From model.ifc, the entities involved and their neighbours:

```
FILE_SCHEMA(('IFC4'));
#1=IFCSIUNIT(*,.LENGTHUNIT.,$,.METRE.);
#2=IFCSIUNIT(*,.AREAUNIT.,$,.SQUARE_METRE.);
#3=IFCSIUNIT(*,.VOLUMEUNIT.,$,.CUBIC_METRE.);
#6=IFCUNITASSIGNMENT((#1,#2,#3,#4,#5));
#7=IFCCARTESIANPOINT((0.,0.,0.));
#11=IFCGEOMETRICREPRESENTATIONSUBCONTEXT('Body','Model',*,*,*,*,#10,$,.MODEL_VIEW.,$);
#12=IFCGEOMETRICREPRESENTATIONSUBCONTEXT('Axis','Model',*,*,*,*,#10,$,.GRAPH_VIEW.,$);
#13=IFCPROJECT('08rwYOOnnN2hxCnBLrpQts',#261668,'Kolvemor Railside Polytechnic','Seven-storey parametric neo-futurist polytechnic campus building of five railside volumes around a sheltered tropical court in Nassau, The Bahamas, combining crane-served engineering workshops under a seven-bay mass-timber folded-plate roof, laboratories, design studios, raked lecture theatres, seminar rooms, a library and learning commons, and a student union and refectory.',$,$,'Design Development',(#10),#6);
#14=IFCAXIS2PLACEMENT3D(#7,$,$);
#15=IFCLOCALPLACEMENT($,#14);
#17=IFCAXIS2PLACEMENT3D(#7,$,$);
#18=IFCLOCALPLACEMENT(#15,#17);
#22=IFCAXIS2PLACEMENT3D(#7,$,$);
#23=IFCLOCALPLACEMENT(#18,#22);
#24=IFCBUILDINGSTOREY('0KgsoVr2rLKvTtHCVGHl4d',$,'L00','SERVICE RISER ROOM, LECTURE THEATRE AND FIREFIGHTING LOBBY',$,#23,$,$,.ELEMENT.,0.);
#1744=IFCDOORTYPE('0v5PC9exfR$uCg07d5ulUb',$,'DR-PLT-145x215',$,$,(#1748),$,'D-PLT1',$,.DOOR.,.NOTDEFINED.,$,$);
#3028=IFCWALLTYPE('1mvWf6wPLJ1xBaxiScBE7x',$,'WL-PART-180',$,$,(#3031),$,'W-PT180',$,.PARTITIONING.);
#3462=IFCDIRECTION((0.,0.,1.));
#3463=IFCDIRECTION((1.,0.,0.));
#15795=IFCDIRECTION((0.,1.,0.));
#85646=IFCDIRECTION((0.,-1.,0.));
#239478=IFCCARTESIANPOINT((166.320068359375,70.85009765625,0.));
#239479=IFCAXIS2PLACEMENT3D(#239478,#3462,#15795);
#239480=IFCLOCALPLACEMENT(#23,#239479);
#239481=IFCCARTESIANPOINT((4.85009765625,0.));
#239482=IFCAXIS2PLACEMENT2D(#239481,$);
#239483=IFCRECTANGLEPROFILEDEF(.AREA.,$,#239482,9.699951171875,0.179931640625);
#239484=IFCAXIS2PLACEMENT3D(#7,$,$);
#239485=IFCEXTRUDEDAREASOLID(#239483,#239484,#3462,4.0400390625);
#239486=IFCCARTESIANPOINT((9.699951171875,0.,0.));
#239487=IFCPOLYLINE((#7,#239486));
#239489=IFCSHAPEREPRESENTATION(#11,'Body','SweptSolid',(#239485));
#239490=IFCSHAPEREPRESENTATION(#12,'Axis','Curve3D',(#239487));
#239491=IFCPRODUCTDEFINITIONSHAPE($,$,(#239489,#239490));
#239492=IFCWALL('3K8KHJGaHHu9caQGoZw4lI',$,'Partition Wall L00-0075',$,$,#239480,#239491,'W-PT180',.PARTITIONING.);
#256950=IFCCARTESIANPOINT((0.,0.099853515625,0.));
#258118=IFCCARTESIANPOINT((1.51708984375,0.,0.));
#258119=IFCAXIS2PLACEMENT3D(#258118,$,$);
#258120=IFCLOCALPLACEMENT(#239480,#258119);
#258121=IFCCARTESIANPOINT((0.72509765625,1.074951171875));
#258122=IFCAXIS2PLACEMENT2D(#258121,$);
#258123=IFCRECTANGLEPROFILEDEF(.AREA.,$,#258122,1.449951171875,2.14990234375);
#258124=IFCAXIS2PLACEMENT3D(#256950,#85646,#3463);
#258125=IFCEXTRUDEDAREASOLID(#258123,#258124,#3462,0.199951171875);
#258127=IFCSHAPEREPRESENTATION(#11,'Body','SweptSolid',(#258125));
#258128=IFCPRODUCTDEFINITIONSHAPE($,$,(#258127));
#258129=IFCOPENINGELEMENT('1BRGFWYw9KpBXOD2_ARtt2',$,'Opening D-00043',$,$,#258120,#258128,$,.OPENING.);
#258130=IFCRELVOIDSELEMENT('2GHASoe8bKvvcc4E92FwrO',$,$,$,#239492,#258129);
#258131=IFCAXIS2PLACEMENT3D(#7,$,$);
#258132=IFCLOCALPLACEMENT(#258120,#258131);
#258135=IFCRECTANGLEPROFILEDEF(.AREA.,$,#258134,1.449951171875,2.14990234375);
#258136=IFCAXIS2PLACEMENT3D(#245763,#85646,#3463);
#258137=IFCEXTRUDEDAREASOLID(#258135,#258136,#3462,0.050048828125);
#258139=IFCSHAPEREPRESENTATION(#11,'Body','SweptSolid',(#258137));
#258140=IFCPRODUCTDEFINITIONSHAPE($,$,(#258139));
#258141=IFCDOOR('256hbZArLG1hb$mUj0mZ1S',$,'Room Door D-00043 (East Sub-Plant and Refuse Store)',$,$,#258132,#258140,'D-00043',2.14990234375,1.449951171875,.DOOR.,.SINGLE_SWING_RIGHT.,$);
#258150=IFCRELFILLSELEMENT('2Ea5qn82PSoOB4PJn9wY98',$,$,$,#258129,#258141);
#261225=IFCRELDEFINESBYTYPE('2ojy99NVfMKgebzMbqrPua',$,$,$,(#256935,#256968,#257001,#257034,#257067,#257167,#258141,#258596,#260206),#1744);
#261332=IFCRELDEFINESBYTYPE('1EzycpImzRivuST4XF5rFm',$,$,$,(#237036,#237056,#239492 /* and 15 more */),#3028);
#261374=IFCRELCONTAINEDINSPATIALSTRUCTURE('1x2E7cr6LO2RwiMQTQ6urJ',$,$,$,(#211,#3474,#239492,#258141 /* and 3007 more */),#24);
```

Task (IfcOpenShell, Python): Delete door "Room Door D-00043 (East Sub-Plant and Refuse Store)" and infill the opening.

```python
import ifcopenshell
import ifcopenshell.api.feature
import ifcopenshell.api.root
import ifcopenshell.geom
import ifcopenshell.util.shape

model = ifcopenshell.open("model.ifc")
settings = ifcopenshell.geom.settings()


def volume(element):
    """Net volume in cubic metres, openings subtracted."""
    shape = ifcopenshell.geom.create_shape(settings, element)
    return ifcopenshell.util.shape.get_volume(shape.geometry)


door = model.by_id(258141)
opening = door.FillsVoids[0].RelatingOpeningElement
wall = opening.VoidsElements[0].RelatingBuildingElement
before = volume(wall)

ifcopenshell.api.root.remove_product(model, product=door)
ifcopenshell.api.feature.remove_feature(model, feature=opening)

after = volume(wall)

print(f"wall volume {before:.3f} -> {after:.3f} m3")

model.write("model_rev.ifc")
```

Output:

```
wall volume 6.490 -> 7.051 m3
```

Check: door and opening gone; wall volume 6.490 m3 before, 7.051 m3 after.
